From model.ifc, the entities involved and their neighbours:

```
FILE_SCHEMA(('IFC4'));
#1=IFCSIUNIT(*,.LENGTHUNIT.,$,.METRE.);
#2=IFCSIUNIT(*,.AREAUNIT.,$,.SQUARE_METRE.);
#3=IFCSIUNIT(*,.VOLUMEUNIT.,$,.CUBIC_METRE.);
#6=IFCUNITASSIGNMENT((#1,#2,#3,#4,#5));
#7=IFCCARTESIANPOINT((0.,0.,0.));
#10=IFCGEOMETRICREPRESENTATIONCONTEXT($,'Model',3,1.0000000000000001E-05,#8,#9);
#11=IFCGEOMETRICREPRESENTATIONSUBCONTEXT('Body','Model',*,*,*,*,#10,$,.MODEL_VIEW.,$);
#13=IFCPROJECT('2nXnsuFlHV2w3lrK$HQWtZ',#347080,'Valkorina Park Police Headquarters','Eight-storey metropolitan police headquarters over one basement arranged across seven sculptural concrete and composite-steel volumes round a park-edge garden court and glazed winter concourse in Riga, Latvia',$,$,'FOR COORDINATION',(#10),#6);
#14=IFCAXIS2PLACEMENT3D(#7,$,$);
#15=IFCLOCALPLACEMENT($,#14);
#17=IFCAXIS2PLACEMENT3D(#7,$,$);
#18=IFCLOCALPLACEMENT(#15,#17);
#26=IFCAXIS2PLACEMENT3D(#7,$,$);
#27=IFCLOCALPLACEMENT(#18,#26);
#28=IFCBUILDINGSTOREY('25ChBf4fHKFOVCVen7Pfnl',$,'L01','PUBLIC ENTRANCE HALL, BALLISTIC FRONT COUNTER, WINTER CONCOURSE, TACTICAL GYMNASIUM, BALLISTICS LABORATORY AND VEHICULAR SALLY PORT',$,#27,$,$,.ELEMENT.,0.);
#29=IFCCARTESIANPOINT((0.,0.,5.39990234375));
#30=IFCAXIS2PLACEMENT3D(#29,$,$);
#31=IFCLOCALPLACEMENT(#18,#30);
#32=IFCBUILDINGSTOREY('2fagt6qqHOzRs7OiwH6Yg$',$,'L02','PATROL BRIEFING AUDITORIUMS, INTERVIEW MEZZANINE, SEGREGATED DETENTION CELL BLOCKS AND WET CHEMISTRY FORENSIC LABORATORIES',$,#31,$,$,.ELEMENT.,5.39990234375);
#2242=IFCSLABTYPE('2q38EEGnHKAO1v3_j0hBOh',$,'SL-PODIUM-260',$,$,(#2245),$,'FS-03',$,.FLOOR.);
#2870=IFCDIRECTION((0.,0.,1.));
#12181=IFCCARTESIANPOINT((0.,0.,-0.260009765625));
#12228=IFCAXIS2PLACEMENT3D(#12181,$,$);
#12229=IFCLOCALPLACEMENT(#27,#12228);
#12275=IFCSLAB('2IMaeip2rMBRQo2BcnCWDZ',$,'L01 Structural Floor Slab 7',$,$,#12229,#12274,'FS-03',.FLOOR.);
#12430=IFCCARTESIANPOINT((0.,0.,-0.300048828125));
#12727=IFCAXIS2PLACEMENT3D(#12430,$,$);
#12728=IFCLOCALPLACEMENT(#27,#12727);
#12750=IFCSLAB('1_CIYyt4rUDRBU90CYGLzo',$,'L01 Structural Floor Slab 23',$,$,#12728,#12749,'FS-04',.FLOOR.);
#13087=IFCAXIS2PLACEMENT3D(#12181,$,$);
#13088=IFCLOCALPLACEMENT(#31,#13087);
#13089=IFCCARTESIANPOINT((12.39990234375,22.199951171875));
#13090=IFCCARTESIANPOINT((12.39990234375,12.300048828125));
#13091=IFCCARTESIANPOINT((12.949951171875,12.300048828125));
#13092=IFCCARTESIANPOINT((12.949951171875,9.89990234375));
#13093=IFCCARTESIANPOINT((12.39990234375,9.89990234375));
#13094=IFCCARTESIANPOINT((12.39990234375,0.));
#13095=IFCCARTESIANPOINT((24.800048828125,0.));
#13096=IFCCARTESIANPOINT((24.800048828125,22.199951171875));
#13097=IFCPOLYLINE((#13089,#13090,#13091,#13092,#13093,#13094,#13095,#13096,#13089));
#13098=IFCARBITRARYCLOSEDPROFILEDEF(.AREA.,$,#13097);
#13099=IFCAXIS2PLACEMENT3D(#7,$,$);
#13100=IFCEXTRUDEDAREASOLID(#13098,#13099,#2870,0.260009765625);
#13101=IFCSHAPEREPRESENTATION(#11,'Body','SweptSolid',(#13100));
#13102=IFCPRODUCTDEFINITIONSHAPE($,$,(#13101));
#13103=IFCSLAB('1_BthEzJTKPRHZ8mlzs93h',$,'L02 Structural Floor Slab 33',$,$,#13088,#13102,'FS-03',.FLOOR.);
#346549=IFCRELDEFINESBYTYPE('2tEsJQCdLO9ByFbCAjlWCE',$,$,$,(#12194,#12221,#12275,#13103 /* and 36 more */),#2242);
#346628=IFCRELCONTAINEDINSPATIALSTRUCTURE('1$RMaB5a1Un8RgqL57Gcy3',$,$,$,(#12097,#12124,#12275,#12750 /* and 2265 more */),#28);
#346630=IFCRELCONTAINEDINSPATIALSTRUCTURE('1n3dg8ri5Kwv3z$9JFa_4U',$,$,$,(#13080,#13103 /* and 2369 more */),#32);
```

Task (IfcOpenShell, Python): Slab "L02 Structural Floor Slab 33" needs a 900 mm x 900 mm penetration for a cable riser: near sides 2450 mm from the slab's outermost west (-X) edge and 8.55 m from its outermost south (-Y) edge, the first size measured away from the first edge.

```python
import numpy as np
import ifcopenshell
import ifcopenshell.api.feature
import ifcopenshell.api.geometry
import ifcopenshell.api.root
import ifcopenshell.geom
import ifcopenshell.util.placement
import ifcopenshell.util.representation
import ifcopenshell.util.shape
import ifcopenshell.util.unit

model = ifcopenshell.open("model.ifc")
unit_scale = ifcopenshell.util.unit.calculate_unit_scale(model)
settings = ifcopenshell.geom.settings()


def volume(element):
    """Net volume in cubic metres, openings subtracted."""
    shape = ifcopenshell.geom.create_shape(settings, element)
    return ifcopenshell.util.shape.get_volume(shape.geometry)


slab = model.by_guid("1_BthEzJTKPRHZ8mlzs93h")
before = volume(slab)

# Extent in the slab's own axes, in metres. The edges named are its -X and -Y sides.
slab_shape = ifcopenshell.geom.create_shape(settings, slab)
vertices = ifcopenshell.util.shape.get_vertices(slab_shape.geometry)
x_min, y_min, bottom = vertices.min(axis=0)
top = vertices[:, 2].max()

opening = ifcopenshell.api.root.create_entity(model, ifc_class="IfcOpeningElement", name="Cable riser opening", predefined_type="OPENING")
context = ifcopenshell.util.representation.get_context(model, "Model", "Body", "MODEL_VIEW")
width, depth = 0.9, 0.9
outline = [(0.0, 0.0), (width, 0.0), (width, depth), (0.0, depth), (0.0, 0.0)]
# Overshoot both faces by 50 mm so the cut is clean.
shape = ifcopenshell.api.geometry.add_slab_representation(
    model, context=context, depth=top - bottom + 0.1, polyline=outline
)
ifcopenshell.api.geometry.assign_representation(model, product=opening, representation=shape)

matrix = ifcopenshell.util.placement.get_local_placement(slab.ObjectPlacement)
matrix[:, 3] = matrix @ np.append(np.array([x_min + 2.45, y_min + 8.55, bottom - 0.05]) / unit_scale, 1.0)
ifcopenshell.api.geometry.edit_object_placement(model, product=opening, matrix=matrix, is_si=False)
ifcopenshell.api.feature.add_feature(model, feature=opening, element=slab)

after = volume(slab)

print(f"slab volume {before:.3f} -> {after:.3f} m3")

model.write("model_v2.ifc")
```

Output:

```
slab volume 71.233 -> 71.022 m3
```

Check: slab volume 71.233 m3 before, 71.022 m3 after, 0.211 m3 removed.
